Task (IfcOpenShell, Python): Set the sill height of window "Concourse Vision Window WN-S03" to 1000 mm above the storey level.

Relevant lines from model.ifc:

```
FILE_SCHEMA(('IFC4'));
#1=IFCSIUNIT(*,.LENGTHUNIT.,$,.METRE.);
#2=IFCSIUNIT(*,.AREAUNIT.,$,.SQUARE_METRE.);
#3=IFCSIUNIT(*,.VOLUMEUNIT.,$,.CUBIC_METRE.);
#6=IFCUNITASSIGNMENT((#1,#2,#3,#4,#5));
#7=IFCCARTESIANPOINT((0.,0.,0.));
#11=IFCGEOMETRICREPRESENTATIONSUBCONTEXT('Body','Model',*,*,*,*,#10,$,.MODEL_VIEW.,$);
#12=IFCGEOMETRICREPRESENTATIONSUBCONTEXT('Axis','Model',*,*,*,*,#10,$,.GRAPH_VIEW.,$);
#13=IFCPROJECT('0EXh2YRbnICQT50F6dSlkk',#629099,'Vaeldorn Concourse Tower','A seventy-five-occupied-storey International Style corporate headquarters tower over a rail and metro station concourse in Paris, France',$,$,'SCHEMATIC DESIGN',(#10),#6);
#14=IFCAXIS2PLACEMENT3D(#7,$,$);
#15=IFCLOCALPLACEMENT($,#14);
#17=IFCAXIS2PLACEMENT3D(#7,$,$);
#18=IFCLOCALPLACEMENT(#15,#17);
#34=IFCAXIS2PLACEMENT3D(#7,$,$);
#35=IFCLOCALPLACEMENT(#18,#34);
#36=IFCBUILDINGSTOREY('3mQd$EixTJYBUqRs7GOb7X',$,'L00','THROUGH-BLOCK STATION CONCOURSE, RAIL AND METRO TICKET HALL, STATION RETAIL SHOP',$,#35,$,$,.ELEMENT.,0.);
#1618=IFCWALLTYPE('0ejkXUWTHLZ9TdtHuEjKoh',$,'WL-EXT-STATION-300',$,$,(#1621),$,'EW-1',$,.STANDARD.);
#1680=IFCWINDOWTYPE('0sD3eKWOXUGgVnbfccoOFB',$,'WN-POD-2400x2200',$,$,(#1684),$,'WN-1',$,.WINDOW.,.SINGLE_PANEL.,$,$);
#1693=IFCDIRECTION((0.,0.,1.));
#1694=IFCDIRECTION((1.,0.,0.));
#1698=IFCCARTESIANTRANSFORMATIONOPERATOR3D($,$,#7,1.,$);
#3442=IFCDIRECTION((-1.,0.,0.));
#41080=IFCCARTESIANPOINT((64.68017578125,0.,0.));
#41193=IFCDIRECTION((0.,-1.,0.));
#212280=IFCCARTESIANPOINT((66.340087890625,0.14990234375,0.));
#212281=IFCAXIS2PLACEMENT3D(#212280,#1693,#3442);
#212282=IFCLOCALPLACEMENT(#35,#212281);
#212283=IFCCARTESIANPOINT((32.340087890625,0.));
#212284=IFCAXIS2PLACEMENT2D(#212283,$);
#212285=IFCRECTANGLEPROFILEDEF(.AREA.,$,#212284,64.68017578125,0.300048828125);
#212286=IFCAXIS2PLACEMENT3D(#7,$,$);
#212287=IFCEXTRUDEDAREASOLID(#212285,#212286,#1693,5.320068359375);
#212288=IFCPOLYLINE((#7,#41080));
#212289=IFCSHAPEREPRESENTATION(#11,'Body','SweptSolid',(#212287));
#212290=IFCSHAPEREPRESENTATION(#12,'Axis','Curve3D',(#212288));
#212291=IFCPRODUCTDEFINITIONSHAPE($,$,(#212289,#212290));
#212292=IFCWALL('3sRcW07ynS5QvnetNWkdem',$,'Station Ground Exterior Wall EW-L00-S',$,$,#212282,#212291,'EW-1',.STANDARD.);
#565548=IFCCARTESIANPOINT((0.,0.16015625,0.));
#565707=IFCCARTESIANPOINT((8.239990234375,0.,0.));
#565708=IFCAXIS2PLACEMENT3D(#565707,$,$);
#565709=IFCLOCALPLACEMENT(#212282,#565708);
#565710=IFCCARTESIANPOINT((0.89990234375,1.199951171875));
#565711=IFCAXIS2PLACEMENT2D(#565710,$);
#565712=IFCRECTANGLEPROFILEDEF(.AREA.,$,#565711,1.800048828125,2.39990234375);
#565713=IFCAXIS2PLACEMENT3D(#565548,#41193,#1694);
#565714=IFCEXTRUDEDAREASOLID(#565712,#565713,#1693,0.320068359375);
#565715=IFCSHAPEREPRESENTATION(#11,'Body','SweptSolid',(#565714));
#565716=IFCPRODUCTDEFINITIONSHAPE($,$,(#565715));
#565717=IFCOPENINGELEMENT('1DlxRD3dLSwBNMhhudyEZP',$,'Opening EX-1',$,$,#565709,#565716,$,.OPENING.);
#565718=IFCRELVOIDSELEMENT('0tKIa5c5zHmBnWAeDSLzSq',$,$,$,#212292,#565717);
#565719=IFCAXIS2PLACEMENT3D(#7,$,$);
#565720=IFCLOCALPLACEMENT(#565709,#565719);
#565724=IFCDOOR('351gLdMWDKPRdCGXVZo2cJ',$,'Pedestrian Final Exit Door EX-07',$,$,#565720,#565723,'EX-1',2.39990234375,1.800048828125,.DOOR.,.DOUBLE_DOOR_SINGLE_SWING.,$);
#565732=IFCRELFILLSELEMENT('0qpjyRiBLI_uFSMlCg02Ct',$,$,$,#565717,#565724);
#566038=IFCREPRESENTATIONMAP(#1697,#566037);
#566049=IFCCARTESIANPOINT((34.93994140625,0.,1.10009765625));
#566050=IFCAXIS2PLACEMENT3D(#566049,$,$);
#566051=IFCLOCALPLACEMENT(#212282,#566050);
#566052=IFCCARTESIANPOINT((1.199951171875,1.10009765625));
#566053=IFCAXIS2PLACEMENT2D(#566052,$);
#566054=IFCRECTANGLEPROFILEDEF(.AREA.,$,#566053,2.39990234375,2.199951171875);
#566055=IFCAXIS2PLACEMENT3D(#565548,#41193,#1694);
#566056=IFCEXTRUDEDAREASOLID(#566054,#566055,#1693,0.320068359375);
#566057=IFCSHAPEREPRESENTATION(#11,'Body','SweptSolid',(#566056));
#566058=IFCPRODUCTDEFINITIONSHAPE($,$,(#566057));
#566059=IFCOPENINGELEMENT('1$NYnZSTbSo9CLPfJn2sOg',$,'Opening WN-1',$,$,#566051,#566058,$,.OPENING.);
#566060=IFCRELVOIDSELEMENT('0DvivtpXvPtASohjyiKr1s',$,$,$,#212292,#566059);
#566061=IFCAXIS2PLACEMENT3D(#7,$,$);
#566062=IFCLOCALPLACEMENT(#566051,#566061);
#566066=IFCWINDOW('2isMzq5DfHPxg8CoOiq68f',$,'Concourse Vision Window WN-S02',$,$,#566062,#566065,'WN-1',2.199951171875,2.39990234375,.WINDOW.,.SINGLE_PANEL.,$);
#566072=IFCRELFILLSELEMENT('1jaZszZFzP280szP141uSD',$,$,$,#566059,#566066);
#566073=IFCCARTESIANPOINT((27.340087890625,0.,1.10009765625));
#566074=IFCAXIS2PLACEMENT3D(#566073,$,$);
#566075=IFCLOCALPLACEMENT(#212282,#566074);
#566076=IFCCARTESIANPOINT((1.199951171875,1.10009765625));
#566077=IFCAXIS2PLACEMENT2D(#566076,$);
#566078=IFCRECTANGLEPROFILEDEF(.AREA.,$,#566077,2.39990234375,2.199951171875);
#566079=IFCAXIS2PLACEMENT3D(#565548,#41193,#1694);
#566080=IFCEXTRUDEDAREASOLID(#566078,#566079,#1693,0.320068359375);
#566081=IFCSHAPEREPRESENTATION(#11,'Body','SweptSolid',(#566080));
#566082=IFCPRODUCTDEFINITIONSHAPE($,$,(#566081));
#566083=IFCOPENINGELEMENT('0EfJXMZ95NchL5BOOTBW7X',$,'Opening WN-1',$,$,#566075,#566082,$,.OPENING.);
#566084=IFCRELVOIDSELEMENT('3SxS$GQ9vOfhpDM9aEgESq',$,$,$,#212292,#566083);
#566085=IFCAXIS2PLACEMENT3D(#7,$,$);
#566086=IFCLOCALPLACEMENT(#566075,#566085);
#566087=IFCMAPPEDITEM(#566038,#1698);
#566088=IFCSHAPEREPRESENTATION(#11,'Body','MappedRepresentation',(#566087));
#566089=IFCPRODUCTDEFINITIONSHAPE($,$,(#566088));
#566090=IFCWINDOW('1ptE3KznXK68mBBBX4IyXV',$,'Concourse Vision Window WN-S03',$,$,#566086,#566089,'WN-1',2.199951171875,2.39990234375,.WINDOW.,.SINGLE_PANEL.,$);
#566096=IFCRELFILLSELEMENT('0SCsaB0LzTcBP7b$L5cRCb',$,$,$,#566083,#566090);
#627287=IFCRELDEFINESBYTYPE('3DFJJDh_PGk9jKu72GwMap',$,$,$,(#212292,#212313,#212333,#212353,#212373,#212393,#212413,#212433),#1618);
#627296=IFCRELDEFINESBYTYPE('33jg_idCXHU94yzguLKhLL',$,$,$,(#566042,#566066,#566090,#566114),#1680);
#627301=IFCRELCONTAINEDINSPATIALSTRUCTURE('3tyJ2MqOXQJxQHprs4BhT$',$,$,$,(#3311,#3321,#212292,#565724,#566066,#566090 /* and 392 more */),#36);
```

```python
import numpy as np
import ifcopenshell
import ifcopenshell.api.geometry
import ifcopenshell.geom
import ifcopenshell.util.element
import ifcopenshell.util.placement
import ifcopenshell.util.shape
import ifcopenshell.util.unit

model = ifcopenshell.open("model.ifc")
unit_scale = ifcopenshell.util.unit.calculate_unit_scale(model)

window = model.by_guid("1ptE3KznXK68mBBBX4IyXV")
opening = window.FillsVoids[0].RelatingOpeningElement
storey = ifcopenshell.util.element.get_container(window, ifc_class="IfcBuildingStorey")
level = ifcopenshell.util.placement.get_local_placement(storey.ObjectPlacement)[2, 3]

# The opening's origin need not be at the sill, so measure its lowest point.
shape = ifcopenshell.geom.create_shape(ifcopenshell.geom.settings(), opening)
bottom = ifcopenshell.util.shape.get_shape_bottom_elevation(shape, shape.geometry) / unit_scale
dz = level + 1.0 - bottom

shift = np.array([0.0, 0.0, dz])
# The window is placed relative to its opening, so it follows when the opening moves.
matrix = ifcopenshell.util.placement.get_local_placement(opening.ObjectPlacement)
matrix[:3, 3] += shift
ifcopenshell.api.geometry.edit_object_placement(
    model, product=opening, matrix=matrix, is_si=False, should_transform_children=True
)

print(f"moved by {dz * unit_scale:+.3f} m")

model.write("model-out.ifc")
```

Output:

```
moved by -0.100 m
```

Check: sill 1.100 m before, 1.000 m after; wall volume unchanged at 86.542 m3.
